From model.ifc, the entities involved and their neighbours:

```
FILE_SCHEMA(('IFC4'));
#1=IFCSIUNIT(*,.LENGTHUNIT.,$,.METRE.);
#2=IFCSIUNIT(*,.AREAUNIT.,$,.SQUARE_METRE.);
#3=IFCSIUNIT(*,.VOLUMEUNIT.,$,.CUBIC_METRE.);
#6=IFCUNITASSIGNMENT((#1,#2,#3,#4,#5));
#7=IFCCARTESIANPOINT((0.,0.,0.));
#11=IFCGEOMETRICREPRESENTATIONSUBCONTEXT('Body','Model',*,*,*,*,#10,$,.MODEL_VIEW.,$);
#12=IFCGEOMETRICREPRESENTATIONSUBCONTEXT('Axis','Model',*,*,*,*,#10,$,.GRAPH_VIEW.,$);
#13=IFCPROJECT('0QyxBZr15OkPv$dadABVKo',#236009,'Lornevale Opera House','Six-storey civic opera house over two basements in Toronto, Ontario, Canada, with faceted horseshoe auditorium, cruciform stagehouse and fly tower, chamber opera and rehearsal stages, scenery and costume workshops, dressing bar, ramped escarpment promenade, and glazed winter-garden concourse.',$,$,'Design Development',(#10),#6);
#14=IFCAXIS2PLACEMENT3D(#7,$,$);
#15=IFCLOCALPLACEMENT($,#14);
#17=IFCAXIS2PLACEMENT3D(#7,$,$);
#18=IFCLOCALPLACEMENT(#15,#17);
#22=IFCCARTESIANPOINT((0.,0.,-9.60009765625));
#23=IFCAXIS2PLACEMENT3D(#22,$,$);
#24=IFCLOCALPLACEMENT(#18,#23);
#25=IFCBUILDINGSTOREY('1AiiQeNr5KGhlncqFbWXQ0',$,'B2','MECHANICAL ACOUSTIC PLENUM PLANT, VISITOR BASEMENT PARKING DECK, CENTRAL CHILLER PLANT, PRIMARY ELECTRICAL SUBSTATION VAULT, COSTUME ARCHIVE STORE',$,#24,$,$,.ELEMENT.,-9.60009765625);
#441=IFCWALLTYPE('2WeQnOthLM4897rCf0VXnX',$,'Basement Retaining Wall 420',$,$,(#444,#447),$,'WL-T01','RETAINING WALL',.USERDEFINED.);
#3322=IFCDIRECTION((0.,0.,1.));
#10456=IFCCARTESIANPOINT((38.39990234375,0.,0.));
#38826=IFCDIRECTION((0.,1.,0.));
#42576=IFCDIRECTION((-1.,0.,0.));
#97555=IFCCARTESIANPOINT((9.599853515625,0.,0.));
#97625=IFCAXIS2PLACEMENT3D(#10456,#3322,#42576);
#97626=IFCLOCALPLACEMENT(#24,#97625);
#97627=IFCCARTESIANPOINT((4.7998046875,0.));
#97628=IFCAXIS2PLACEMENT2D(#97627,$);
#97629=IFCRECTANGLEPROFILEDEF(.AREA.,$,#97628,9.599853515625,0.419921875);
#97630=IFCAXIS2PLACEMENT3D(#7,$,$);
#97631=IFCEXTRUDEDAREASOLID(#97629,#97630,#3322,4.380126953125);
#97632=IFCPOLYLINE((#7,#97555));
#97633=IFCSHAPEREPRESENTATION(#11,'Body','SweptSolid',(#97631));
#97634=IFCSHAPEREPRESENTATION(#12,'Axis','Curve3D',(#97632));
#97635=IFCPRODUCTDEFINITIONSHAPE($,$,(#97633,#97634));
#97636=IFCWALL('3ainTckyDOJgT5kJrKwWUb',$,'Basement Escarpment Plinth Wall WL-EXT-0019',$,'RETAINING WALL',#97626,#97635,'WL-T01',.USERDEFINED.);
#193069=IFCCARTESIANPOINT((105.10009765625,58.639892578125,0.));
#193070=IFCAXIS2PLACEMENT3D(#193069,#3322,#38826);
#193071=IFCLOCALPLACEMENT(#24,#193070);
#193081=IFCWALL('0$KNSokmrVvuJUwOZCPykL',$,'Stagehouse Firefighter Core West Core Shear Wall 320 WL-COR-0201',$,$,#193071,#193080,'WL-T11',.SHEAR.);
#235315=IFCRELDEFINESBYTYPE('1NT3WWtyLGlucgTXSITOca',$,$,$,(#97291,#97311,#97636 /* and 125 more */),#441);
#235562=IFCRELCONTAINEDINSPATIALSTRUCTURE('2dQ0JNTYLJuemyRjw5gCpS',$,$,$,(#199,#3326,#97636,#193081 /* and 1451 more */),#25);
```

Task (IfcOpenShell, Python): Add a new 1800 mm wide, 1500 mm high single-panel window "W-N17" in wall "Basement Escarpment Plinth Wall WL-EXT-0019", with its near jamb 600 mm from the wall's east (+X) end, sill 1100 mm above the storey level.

```python
import numpy as np
import ifcopenshell
import ifcopenshell.api.feature
import ifcopenshell.api.geometry
import ifcopenshell.api.root
import ifcopenshell.api.spatial
import ifcopenshell.geom
import ifcopenshell.util.element
import ifcopenshell.util.placement
import ifcopenshell.util.representation
import ifcopenshell.util.shape
import ifcopenshell.util.unit

model = ifcopenshell.open("model.ifc")
unit_scale = ifcopenshell.util.unit.calculate_unit_scale(model)
settings = ifcopenshell.geom.settings()


def volume(element):
    """Net volume in cubic metres, openings subtracted."""
    shape = ifcopenshell.geom.create_shape(settings, element)
    return ifcopenshell.util.shape.get_volume(shape.geometry)


wall = model.by_guid("3ainTckyDOJgT5kJrKwWUb")
storey = ifcopenshell.util.element.get_container(wall, ifc_class="IfcBuildingStorey")
context = ifcopenshell.util.representation.get_context(model, "Model", "Body", "MODEL_VIEW")
before = volume(wall)

width, height, from_end, sill = 1.8, 1.5, 0.6, 1.1  # metres

# The wall runs along its own X axis, and the end named is its -X end.
wall_shape = ifcopenshell.geom.create_shape(settings, wall)
x, y, z = ifcopenshell.util.shape.get_vertices(wall_shape.geometry).T
start = x.min() + from_end
face, thickness = float(y.min()), float(y.max() - y.min())
wall_matrix = ifcopenshell.util.placement.get_local_placement(wall.ObjectPlacement)
level = ifcopenshell.util.placement.get_local_placement(storey.ObjectPlacement)[2, 3]


def in_wall(x, y):
    """Placement at x, y metres in the wall's axes, at sill height."""
    matrix = wall_matrix.copy()
    matrix[:, 3] = wall_matrix @ np.array([x / unit_scale, y / unit_scale, 0.0, 1.0])
    matrix[2, 3] = level + sill / unit_scale
    return matrix


# Opening: a box that overshoots both wall faces by 50 mm.
opening = ifcopenshell.api.root.create_entity(model, ifc_class="IfcOpeningElement", predefined_type="OPENING")
box = ifcopenshell.api.geometry.add_wall_representation(
    model, context=context, length=width, height=height, thickness=thickness + 0.1
)
ifcopenshell.api.geometry.assign_representation(model, product=opening, representation=box)
ifcopenshell.api.geometry.edit_object_placement(model, product=opening, matrix=in_wall(start, face - 0.05), is_si=False)
ifcopenshell.api.feature.add_feature(model, feature=opening, element=wall)

window = ifcopenshell.api.root.create_entity(model, ifc_class="IfcWindow", name="W-N17", predefined_type="WINDOW")
window.OverallWidth, window.OverallHeight = width / unit_scale, height / unit_scale
window.PartitioningType = "SINGLE_PANEL"
body = ifcopenshell.api.geometry.add_window_representation(
    model,
    context=context,
    overall_width=window.OverallWidth,
    overall_height=window.OverallHeight,
    partition_type="SINGLE_PANEL",
)
ifcopenshell.api.geometry.assign_representation(model, product=window, representation=body)
ifcopenshell.api.spatial.assign_container(model, products=[window], relating_structure=storey)
ifcopenshell.api.feature.add_filling(model, opening=opening, element=window)

# Centre the window in the wall's thickness.
ifcopenshell.api.geometry.edit_object_placement(model, product=window, matrix=in_wall(start, face), is_si=False)
window_shape = ifcopenshell.geom.create_shape(settings, window)
depth = ifcopenshell.util.shape.get_vertices(window_shape.geometry)[:, 1]
offset = face + thickness / 2 - (depth.min() + depth.max()) / 2
ifcopenshell.api.geometry.edit_object_placement(model, product=window, matrix=in_wall(start, offset), is_si=False)

after = volume(wall)

print(f"wall volume {before:.3f} -> {after:.3f} m3")

model.write("model_v2.ifc")
```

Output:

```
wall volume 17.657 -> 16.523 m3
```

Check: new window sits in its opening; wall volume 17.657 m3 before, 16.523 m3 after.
